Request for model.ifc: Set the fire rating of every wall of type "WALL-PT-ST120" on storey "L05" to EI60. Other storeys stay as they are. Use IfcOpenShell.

First a look at what the model holds.

```python
import ifcopenshell
import ifcopenshell.util.element

model = ifcopenshell.open("model.ifc")
print(model.schema)
storey = next(s for s in model.by_type("IfcBuildingStorey") if s.Name == "L05")
walls = [e for e in ifcopenshell.util.element.get_decomposition(storey) if e.is_a("IfcWall")]
seen = {}
for e in walls:
    element_type = ifcopenshell.util.element.get_type(e)
    key = (element_type.Name if element_type != e and element_type else None, ifcopenshell.util.element.get_pset(e, "Pset_WallCommon", "FireRating"))
    seen[key] = seen.get(key, 0) + 1
for (name, value), count in sorted(seen.items(), key=str):
    print(count, "x", name, "|", value)
```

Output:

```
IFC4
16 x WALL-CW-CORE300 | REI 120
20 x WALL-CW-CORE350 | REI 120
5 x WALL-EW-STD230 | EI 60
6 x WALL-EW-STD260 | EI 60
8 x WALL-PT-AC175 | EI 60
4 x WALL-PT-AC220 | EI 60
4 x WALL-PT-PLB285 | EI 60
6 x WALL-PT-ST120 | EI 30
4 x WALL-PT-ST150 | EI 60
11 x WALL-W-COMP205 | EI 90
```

```python
import ifcopenshell
import ifcopenshell.api.pset
import ifcopenshell.util.element

model = ifcopenshell.open("model.ifc")

storey = next(s for s in model.by_type("IfcBuildingStorey") if s.Name == "L05")
walls = [e for e in ifcopenshell.util.element.get_decomposition(storey) if e.is_a("IfcWall")]

count = 0
for e in walls:
    element_type = ifcopenshell.util.element.get_type(e)
    if element_type in (None, e) or element_type.Name != "WALL-PT-ST120":
        continue
    # add_pset returns the element's existing set when there is one.
    pset = ifcopenshell.api.pset.add_pset(model, product=e, name="Pset_WallCommon")
    ifcopenshell.api.pset.edit_pset(model, pset=pset, properties={"FireRating": "EI60"})
    count += 1

print(count, "walls updated")

model.write("model_rev.ifc")
```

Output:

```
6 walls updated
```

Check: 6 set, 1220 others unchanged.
